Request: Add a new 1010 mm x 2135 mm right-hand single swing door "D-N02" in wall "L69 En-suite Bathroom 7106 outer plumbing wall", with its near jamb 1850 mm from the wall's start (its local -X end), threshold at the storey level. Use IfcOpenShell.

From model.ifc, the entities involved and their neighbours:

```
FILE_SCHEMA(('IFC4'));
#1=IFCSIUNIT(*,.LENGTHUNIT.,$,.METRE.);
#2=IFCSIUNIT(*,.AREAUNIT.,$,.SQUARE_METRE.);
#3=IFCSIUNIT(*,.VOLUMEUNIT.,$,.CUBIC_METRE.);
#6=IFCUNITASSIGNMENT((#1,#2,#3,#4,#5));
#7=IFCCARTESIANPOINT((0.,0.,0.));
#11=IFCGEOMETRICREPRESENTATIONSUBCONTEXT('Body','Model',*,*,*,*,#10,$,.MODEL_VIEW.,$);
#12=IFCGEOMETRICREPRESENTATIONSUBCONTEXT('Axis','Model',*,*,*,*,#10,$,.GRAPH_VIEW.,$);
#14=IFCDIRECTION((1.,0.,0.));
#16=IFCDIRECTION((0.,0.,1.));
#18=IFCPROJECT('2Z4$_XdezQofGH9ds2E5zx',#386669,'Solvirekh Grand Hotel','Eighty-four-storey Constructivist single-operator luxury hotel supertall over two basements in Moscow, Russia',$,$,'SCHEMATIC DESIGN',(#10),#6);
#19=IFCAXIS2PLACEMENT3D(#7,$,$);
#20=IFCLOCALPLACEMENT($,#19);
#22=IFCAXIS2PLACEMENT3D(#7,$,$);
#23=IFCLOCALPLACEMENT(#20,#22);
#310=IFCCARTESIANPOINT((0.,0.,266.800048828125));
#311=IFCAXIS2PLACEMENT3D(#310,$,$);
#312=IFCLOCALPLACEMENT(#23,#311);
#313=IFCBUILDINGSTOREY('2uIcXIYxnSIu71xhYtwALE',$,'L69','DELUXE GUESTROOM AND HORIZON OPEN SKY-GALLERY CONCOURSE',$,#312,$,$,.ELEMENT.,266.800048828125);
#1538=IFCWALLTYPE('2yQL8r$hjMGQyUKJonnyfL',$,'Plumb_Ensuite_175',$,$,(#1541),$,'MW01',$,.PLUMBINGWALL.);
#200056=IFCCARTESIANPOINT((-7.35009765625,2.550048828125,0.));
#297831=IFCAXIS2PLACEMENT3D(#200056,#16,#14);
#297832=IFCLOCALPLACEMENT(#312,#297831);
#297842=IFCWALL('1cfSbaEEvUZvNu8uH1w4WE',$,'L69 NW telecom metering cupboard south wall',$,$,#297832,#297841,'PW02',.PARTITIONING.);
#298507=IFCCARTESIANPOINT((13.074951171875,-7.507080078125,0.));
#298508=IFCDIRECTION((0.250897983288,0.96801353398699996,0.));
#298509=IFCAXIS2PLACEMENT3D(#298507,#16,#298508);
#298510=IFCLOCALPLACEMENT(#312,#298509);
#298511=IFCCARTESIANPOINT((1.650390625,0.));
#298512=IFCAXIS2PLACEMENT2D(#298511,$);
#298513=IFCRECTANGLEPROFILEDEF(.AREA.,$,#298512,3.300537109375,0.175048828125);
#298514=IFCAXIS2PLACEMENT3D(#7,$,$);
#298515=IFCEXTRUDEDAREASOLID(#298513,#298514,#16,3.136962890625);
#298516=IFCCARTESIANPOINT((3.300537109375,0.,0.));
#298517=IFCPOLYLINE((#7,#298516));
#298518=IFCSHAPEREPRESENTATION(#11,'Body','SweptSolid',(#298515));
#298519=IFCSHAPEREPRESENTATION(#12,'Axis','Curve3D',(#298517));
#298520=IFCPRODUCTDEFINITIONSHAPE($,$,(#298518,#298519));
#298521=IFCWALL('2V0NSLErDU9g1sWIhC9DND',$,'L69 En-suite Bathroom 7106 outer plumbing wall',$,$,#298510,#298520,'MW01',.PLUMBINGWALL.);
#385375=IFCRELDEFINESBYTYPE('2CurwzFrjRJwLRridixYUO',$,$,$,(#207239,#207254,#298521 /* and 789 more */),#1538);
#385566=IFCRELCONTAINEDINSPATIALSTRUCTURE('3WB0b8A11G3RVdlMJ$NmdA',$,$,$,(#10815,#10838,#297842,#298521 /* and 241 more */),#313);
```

```python
import numpy as np
import ifcopenshell
import ifcopenshell.api.feature
import ifcopenshell.api.geometry
import ifcopenshell.api.root
import ifcopenshell.api.spatial
import ifcopenshell.geom
import ifcopenshell.util.element
import ifcopenshell.util.placement
import ifcopenshell.util.representation
import ifcopenshell.util.shape
import ifcopenshell.util.unit

model = ifcopenshell.open("model.ifc")
unit_scale = ifcopenshell.util.unit.calculate_unit_scale(model)
settings = ifcopenshell.geom.settings()


def volume(element):
    """Net volume in cubic metres, openings subtracted."""
    shape = ifcopenshell.geom.create_shape(settings, element)
    return ifcopenshell.util.shape.get_volume(shape.geometry)


wall = model.by_id(298521)
storey = ifcopenshell.util.element.get_container(wall, ifc_class="IfcBuildingStorey")
context = ifcopenshell.util.representation.get_context(model, "Model", "Body", "MODEL_VIEW")
before = volume(wall)

width, height, from_end, sill = 1.01, 2.135, 1.85, 0.0  # metres

# The wall runs along its own X axis, and the end named is its -X end.
wall_shape = ifcopenshell.geom.create_shape(settings, wall)
x, y, z = ifcopenshell.util.shape.get_vertices(wall_shape.geometry).T
start = x.min() + from_end
face, thickness = float(y.min()), float(y.max() - y.min())
wall_matrix = ifcopenshell.util.placement.get_local_placement(wall.ObjectPlacement)
level = ifcopenshell.util.placement.get_local_placement(storey.ObjectPlacement)[2, 3]


def in_wall(x, y):
    """Placement at x, y metres in the wall's axes, at sill height."""
    matrix = wall_matrix.copy()
    matrix[:, 3] = wall_matrix @ np.array([x / unit_scale, y / unit_scale, 0.0, 1.0])
    matrix[2, 3] = level + sill / unit_scale
    return matrix


# Opening: a box that overshoots both wall faces by 50 mm.
opening = ifcopenshell.api.root.create_entity(model, ifc_class="IfcOpeningElement", predefined_type="OPENING")
box = ifcopenshell.api.geometry.add_wall_representation(
    model, context=context, length=width, height=height, thickness=thickness + 0.1
)
ifcopenshell.api.geometry.assign_representation(model, product=opening, representation=box)
ifcopenshell.api.geometry.edit_object_placement(model, product=opening, matrix=in_wall(start, face - 0.05), is_si=False)
ifcopenshell.api.feature.add_feature(model, feature=opening, element=wall)

door = ifcopenshell.api.root.create_entity(model, ifc_class="IfcDoor", name="D-N02", predefined_type="DOOR")
door.OverallWidth, door.OverallHeight = width / unit_scale, height / unit_scale
door.OperationType = "SINGLE_SWING_RIGHT"
body = ifcopenshell.api.geometry.add_door_representation(
    model,
    context=context,
    overall_width=door.OverallWidth,
    overall_height=door.OverallHeight,
    operation_type="SINGLE_SWING_RIGHT",
    lining_properties={"LiningDepth": thickness / unit_scale, "ThresholdDepth": thickness / unit_scale},
)
ifcopenshell.api.geometry.assign_representation(model, product=door, representation=body)
ifcopenshell.api.spatial.assign_container(model, products=[door], relating_structure=storey)
ifcopenshell.api.feature.add_filling(model, opening=opening, element=door)

# The lining spans the wall, so the door starts at the wall face.
ifcopenshell.api.geometry.edit_object_placement(model, product=door, matrix=in_wall(start, face), is_si=False)

after = volume(wall)

print(f"wall volume {before:.3f} -> {after:.3f} m3")

model.write("model_edited.ifc")
```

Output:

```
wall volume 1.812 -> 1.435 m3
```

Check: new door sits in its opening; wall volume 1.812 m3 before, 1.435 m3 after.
